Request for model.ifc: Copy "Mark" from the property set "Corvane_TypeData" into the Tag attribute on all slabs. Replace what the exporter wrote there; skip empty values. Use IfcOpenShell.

First a look at what the model holds.

```python
import ifcopenshell
import ifcopenshell.util.element

model = ifcopenshell.open("model.ifc")
print(model.schema)
slabs = model.by_type("IfcSlab")
print(len(slabs), "slabs")
for e in slabs[:8]:
    source = ifcopenshell.util.element.get_pset(e, "Corvane_TypeData", "Mark")
    target = e.Tag
    print(e.id(), repr(source), repr(target), sep=" | ")
```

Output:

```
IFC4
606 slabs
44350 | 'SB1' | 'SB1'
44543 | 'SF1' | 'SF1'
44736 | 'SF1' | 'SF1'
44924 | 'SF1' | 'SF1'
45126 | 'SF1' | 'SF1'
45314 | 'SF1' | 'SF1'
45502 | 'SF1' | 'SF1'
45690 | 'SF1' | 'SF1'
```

```python
import ifcopenshell
import ifcopenshell.util.element

model = ifcopenshell.open("model.ifc")

count = 0
for e in model.by_type("IfcSlab"):
    value = ifcopenshell.util.element.get_pset(e, "Corvane_TypeData", "Mark")
    current = e.Tag
    if not value or not value.strip() or current == value:
        continue
    e.Tag = value
    count += 1

print(count, "slabs updated")

model.write("model_rev.ifc")
```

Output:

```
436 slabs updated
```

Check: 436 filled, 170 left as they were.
